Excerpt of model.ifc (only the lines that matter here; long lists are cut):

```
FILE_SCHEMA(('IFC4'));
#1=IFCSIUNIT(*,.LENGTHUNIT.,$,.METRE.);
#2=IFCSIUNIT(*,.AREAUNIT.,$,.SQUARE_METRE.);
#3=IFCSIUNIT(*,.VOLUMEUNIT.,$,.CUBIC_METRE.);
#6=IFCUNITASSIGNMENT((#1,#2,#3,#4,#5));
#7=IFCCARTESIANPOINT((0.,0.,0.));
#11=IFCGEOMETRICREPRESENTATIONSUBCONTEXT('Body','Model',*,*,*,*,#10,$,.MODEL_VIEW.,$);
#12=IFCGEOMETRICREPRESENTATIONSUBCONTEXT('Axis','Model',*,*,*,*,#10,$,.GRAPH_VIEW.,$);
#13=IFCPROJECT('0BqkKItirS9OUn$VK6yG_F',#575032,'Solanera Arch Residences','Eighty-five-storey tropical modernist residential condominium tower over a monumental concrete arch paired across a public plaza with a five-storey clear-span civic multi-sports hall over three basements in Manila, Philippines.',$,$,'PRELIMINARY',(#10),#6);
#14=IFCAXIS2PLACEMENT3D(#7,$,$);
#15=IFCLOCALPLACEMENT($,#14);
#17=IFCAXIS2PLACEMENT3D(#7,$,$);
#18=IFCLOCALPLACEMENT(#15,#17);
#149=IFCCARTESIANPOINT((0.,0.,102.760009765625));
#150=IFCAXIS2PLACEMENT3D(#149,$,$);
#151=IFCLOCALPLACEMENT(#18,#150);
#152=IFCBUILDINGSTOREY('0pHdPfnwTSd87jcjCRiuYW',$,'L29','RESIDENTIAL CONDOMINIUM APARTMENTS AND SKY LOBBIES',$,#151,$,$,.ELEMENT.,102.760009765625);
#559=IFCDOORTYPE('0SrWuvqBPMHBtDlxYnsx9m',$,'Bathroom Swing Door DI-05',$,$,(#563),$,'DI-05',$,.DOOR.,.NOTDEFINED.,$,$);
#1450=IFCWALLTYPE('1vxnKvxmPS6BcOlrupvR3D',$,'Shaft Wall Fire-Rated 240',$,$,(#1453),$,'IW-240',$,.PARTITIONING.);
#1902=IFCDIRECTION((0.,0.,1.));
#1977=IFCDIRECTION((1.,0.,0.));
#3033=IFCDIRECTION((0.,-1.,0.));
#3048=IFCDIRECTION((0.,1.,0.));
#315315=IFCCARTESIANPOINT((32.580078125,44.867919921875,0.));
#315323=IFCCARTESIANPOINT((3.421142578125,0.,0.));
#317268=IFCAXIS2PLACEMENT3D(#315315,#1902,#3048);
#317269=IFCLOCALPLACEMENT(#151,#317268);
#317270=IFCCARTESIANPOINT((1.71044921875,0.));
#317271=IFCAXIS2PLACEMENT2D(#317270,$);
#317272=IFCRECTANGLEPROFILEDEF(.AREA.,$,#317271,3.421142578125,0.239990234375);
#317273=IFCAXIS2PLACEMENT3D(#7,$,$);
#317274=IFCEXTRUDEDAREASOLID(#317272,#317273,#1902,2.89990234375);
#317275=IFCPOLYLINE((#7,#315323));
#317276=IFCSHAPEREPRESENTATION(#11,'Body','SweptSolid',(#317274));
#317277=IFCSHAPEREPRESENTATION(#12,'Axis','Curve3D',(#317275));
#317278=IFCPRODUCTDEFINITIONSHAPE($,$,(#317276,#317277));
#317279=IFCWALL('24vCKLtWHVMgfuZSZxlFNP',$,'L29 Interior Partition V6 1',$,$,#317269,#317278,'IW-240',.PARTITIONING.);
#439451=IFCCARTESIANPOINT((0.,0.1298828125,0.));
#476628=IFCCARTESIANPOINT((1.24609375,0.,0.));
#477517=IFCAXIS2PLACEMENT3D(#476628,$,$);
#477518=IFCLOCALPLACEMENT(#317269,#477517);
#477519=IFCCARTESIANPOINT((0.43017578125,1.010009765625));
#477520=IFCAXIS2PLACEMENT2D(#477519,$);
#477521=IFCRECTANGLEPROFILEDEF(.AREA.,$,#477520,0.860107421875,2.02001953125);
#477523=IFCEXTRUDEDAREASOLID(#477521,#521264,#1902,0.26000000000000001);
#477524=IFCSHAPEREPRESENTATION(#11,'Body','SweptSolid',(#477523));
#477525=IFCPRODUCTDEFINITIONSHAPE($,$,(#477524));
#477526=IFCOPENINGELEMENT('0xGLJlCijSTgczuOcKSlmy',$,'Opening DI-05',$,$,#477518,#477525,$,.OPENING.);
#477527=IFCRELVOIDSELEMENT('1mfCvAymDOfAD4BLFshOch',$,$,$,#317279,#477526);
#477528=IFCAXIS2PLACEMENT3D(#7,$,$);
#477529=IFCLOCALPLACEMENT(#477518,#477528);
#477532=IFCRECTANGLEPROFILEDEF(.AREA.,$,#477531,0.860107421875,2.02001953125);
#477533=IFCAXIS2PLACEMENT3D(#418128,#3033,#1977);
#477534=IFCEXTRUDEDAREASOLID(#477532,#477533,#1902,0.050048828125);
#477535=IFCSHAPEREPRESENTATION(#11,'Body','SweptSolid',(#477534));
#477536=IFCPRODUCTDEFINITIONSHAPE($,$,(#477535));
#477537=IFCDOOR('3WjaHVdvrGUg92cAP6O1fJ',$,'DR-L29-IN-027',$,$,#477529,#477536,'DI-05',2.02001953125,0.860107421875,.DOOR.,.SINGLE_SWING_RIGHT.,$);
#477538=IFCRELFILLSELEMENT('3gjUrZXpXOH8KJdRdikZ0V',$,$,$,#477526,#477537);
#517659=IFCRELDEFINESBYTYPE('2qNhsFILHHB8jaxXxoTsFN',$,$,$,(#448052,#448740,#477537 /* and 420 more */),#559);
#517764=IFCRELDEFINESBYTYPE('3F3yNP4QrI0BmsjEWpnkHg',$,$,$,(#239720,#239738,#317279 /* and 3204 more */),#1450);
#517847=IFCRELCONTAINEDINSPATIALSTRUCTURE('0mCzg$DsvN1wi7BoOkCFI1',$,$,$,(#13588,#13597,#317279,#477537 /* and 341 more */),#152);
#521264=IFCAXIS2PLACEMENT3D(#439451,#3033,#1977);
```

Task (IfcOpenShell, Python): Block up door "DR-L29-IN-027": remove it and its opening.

```python
import ifcopenshell
import ifcopenshell.api.feature
import ifcopenshell.api.root
import ifcopenshell.geom
import ifcopenshell.util.shape

model = ifcopenshell.open("model.ifc")
settings = ifcopenshell.geom.settings()


def volume(element):
    """Net volume in cubic metres, openings subtracted."""
    shape = ifcopenshell.geom.create_shape(settings, element)
    return ifcopenshell.util.shape.get_volume(shape.geometry)


door = model.by_guid("3WjaHVdvrGUg92cAP6O1fJ")
opening = door.FillsVoids[0].RelatingOpeningElement
wall = opening.VoidsElements[0].RelatingBuildingElement
before = volume(wall)

ifcopenshell.api.root.remove_product(model, product=door)
ifcopenshell.api.feature.remove_feature(model, feature=opening)

after = volume(wall)

print(f"wall volume {before:.3f} -> {after:.3f} m3")

model.write("model_edited.ifc")
```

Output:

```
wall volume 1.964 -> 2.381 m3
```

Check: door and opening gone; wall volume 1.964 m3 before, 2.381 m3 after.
